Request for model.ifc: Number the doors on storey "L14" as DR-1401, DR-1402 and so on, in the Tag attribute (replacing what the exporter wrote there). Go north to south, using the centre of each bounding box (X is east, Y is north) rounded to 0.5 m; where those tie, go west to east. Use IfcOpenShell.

First a look at what the model holds.

```python
import ifcopenshell
import ifcopenshell.util.element
import ifcopenshell.util.placement

model = ifcopenshell.open("model.ifc")
print(model.schema)
storey = next(s for s in model.by_type("IfcBuildingStorey") if s.Name == "L14")
doors = [e for e in ifcopenshell.util.element.get_decomposition(storey) if e.is_a("IfcDoor")]
for e in sorted(doors, key=lambda e: e.id()):
    origin = ifcopenshell.util.placement.get_local_placement(e.ObjectPlacement)[:3, 3]
    print(e.id(), e.Tag, e.Name, origin.round(2) + 0.0, sep=" | ")
```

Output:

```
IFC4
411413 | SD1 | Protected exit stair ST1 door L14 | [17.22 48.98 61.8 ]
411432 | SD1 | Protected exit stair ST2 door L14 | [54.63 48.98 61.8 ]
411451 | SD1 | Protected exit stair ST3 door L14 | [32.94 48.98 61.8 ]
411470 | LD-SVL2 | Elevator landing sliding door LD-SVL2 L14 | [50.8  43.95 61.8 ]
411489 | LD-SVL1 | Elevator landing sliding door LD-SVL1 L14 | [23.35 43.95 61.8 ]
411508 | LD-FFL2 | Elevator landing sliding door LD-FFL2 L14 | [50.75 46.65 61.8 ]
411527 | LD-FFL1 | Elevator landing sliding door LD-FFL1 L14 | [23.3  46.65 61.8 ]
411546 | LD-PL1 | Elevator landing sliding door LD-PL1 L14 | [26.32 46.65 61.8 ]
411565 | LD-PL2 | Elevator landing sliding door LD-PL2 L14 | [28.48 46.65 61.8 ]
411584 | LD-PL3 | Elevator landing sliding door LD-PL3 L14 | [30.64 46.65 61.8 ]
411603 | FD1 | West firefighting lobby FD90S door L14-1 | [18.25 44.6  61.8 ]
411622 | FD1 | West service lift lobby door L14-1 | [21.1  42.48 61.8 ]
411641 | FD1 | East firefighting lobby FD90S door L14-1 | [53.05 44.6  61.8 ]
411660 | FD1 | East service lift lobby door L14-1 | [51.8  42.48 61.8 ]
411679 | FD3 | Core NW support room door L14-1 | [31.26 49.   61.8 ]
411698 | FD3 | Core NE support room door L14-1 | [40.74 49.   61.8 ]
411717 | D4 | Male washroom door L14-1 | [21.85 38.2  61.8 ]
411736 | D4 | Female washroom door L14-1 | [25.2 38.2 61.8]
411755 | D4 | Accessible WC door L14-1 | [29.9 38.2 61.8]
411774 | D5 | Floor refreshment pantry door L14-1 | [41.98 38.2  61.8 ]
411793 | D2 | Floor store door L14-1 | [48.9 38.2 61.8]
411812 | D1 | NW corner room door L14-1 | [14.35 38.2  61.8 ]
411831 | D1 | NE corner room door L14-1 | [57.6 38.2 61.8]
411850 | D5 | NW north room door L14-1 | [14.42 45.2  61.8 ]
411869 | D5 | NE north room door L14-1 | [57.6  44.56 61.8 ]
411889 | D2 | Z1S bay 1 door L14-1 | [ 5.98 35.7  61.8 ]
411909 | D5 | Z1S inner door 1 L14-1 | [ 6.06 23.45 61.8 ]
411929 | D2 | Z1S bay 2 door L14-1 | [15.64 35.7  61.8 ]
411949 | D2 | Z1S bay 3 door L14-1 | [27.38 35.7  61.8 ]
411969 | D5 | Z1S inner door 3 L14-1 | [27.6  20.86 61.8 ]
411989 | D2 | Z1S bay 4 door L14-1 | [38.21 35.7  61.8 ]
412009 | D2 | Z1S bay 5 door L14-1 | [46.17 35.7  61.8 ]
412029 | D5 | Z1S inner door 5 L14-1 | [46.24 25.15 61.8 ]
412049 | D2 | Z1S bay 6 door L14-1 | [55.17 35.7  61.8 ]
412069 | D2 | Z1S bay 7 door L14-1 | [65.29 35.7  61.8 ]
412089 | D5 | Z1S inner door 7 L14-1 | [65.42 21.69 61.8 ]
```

```python
import ifcopenshell
import ifcopenshell.geom
import ifcopenshell.util.element
import ifcopenshell.util.shape

model = ifcopenshell.open("model.ifc")
settings = ifcopenshell.geom.settings()
settings.set("use-world-coords", True)


def centre(element):
    shape = ifcopenshell.geom.create_shape(settings, element)
    return ifcopenshell.util.shape.get_bbox_centroid(shape.geometry)


storey = next(s for s in model.by_type("IfcBuildingStorey") if s.Name == "L14")
doors = [e for e in ifcopenshell.util.element.get_decomposition(storey) if e.is_a("IfcDoor")]

# Insertion points can sit at a corner or the storey origin, so sort by the geometry (in metres).
centres = {e: centre(e) for e in doors}
doors.sort(key=lambda e: (-round(centres[e][1] / 0.5), centres[e][0]))

for i, e in enumerate(doors, start=1):
    number = f"DR-14{i:02d}"
    e.Tag = number
    print(e.id(), number)

model.write("model_edited.ifc")
```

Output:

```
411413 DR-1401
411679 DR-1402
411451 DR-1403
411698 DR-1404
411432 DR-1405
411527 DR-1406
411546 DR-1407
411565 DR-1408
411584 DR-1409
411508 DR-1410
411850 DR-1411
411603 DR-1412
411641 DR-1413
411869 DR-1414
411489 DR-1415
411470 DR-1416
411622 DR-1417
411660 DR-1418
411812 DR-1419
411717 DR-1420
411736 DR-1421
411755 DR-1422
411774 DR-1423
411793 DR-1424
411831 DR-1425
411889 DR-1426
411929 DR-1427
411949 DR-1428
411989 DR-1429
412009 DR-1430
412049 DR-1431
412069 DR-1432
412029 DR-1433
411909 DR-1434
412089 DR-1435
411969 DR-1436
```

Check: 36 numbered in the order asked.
